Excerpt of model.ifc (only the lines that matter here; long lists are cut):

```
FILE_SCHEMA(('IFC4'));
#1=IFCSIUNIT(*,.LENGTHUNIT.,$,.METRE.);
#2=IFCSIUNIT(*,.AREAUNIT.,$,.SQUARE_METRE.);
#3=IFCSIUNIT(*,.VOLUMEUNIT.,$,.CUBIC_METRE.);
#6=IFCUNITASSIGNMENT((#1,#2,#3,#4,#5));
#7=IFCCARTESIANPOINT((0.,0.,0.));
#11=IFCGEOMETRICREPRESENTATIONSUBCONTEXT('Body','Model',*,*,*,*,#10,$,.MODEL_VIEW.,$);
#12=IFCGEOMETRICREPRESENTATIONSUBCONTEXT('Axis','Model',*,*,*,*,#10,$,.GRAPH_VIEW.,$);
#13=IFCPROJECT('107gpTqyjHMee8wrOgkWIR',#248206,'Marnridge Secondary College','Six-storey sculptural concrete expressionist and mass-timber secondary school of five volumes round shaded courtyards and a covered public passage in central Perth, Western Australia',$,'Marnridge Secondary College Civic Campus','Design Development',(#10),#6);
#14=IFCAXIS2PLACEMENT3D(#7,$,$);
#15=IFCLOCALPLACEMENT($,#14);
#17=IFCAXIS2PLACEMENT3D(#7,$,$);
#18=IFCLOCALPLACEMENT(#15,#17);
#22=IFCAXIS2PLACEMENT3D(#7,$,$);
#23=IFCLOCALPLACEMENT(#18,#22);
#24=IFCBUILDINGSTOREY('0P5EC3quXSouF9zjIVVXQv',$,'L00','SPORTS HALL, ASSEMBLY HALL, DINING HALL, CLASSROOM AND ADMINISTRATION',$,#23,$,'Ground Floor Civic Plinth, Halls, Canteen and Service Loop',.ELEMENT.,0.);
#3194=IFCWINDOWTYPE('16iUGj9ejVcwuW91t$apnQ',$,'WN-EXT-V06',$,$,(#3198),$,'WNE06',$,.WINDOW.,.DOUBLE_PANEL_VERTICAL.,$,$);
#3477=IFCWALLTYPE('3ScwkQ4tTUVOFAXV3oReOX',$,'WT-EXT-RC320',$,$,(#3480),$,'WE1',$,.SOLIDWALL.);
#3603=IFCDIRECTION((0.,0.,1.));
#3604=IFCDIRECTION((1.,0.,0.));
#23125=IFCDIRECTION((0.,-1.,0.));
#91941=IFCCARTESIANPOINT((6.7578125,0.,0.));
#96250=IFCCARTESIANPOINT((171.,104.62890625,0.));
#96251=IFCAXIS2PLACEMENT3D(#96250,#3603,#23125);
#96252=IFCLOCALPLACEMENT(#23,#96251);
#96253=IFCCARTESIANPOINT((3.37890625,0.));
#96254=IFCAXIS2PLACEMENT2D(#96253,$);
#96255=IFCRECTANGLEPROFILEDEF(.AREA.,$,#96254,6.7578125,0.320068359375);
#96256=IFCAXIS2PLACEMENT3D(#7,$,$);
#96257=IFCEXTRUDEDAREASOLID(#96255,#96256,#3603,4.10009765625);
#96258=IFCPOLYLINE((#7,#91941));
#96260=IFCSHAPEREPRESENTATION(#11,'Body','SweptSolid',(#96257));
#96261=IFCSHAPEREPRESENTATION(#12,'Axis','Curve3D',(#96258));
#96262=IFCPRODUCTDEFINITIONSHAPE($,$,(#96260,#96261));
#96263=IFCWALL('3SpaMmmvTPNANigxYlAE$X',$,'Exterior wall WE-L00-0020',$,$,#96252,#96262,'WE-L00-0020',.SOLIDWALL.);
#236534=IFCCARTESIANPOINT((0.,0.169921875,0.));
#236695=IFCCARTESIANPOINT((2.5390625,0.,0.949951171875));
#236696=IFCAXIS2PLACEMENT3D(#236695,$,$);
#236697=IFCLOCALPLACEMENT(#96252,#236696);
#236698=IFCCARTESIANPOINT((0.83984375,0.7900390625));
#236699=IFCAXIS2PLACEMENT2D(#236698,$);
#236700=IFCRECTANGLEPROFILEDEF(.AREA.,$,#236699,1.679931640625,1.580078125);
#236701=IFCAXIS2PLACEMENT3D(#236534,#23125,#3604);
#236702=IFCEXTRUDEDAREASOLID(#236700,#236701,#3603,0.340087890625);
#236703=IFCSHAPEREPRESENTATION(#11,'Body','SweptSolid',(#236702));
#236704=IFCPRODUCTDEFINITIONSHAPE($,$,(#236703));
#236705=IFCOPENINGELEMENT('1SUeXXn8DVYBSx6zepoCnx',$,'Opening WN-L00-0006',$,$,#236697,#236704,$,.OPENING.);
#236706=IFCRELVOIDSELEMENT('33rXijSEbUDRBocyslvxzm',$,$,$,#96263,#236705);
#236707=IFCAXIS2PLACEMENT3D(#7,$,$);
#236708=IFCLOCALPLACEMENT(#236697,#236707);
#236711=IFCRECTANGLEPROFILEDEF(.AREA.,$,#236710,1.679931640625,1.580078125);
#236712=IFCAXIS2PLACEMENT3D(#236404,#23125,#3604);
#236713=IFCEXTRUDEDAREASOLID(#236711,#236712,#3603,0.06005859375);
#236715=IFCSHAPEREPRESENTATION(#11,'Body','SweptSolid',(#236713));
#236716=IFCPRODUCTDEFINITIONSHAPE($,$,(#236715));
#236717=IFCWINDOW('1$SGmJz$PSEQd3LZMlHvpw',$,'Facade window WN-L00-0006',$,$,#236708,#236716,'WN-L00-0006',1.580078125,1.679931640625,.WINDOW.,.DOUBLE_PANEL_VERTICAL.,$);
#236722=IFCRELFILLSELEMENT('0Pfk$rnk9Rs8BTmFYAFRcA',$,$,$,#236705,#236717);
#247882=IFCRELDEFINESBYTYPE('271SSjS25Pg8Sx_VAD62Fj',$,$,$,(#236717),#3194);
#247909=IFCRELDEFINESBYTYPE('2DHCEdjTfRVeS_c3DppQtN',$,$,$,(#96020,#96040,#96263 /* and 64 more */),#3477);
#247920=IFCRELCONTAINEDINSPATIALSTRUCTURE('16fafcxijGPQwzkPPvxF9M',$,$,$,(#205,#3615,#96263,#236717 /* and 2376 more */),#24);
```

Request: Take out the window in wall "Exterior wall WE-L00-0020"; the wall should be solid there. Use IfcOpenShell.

```python
import ifcopenshell
import ifcopenshell.api.feature
import ifcopenshell.api.root
import ifcopenshell.geom
import ifcopenshell.util.shape

model = ifcopenshell.open("model.ifc")
settings = ifcopenshell.geom.settings()


def volume(element):
    """Net volume in cubic metres, openings subtracted."""
    shape = ifcopenshell.geom.create_shape(settings, element)
    return ifcopenshell.util.shape.get_volume(shape.geometry)


window = model.by_id(236717)
opening = window.FillsVoids[0].RelatingOpeningElement
wall = opening.VoidsElements[0].RelatingBuildingElement
before = volume(wall)

ifcopenshell.api.root.remove_product(model, product=window)
ifcopenshell.api.feature.remove_feature(model, feature=opening)

after = volume(wall)

print(f"wall volume {before:.3f} -> {after:.3f} m3")

model.write("model_edited.ifc")
```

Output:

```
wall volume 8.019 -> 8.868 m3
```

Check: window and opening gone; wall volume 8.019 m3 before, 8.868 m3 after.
